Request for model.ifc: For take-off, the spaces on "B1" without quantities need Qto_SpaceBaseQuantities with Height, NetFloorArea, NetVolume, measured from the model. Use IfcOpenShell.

First a look at what the model holds.

```python
import ifcopenshell
import ifcopenshell.util.element
import ifcopenshell.util.unit

model = ifcopenshell.open("model.ifc")
print(model.schema)
for unit_type in ("LENGTHUNIT", "AREAUNIT", "VOLUMEUNIT"):
    print(unit_type, ifcopenshell.util.unit.calculate_unit_scale(model, unit_type))
storey = next(s for s in model.by_type("IfcBuildingStorey") if s.Name == "B1")
spaces = [e for e in ifcopenshell.util.element.get_decomposition(storey) if e.is_a("IfcSpace")]
for e in sorted(spaces, key=lambda e: e.id()):
    print(e.id(), e.is_a(), e.Name, list(ifcopenshell.util.element.get_psets(e, qtos_only=True)), sep=" | ")
```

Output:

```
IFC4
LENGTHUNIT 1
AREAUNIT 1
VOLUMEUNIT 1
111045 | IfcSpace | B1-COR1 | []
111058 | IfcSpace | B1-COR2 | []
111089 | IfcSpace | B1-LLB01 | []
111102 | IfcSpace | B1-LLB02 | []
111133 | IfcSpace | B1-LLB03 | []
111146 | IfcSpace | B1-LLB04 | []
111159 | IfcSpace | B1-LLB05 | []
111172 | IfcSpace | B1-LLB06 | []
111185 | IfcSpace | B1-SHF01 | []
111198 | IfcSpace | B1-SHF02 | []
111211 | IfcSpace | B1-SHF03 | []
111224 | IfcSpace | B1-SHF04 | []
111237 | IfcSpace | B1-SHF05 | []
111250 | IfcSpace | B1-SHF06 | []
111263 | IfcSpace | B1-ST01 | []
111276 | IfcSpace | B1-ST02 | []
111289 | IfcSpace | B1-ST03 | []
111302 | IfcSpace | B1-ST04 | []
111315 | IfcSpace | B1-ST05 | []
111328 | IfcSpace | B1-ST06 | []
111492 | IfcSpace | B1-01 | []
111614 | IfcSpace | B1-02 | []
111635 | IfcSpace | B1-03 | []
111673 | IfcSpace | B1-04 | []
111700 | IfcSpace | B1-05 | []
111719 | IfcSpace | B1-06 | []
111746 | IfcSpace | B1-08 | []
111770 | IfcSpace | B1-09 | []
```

```python
import ifcopenshell
import ifcopenshell.api.pset
import ifcopenshell.geom
import ifcopenshell.util.element
import ifcopenshell.util.shape
import ifcopenshell.util.unit

model = ifcopenshell.open("model.ifc")
unit_scale = ifcopenshell.util.unit.calculate_unit_scale(model)
area_scale = ifcopenshell.util.unit.calculate_unit_scale(model, "AREAUNIT")
volume_scale = ifcopenshell.util.unit.calculate_unit_scale(model, "VOLUMEUNIT")
settings = ifcopenshell.geom.settings()

storey = next(s for s in model.by_type("IfcBuildingStorey") if s.Name == "B1")
spaces = [e for e in ifcopenshell.util.element.get_decomposition(storey) if e.is_a("IfcSpace")]

for e in sorted(spaces, key=lambda e: e.id()):
    if ifcopenshell.util.element.get_psets(e, qtos_only=True, should_inherit=False):
        continue
    # Geometry comes back in metres, in the element's own axes.
    shape = ifcopenshell.geom.create_shape(settings, e)
    values = {
        "Height": ifcopenshell.util.shape.get_z(shape.geometry) / unit_scale,
        "NetFloorArea": ifcopenshell.util.shape.get_footprint_area(shape.geometry) / area_scale,
        "NetVolume": ifcopenshell.util.shape.get_volume(shape.geometry) / volume_scale,
    }
    qto = ifcopenshell.api.pset.add_qto(model, product=e, name="Qto_SpaceBaseQuantities")
    ifcopenshell.api.pset.edit_qto(model, qto=qto, properties=values)
    print(e.id(), {k: round(v, 3) for k, v in values.items()})

model.write("model_edited.ifc")
```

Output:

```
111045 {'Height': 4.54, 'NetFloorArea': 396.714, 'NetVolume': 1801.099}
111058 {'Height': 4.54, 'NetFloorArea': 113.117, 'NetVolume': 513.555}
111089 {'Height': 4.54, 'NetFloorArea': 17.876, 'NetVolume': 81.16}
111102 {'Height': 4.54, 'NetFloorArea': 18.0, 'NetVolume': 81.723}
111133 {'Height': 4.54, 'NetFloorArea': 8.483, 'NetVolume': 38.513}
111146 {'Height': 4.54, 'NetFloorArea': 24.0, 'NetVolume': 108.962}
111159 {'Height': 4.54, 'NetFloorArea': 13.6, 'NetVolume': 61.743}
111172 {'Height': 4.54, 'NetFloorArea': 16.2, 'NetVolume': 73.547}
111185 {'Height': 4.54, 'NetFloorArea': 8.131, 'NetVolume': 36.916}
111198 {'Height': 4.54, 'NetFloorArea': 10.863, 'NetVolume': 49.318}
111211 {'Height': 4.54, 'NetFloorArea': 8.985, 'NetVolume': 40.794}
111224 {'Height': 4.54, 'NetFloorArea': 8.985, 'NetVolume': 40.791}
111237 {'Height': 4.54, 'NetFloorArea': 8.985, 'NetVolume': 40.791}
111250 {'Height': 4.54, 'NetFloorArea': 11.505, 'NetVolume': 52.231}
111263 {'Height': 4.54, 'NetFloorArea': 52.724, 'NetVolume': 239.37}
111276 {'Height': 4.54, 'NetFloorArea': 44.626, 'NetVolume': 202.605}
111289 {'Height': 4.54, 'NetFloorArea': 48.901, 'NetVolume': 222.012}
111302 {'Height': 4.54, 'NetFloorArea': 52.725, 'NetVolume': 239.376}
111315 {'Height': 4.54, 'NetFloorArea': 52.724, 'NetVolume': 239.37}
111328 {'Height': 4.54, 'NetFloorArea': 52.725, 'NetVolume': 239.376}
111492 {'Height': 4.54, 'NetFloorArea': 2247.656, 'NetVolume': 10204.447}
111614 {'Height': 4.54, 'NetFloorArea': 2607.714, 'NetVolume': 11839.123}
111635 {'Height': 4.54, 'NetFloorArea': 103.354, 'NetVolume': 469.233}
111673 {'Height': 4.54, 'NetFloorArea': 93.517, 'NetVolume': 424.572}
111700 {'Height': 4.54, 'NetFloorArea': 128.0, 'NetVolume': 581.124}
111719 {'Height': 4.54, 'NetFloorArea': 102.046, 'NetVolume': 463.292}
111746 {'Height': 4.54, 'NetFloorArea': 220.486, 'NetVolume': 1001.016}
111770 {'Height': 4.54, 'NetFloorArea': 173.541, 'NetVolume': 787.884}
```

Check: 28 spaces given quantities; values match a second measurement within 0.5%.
